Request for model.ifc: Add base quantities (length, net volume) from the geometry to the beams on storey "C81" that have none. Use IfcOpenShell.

First a look at what the model holds.

```python
import ifcopenshell
import ifcopenshell.util.element
import ifcopenshell.util.unit

model = ifcopenshell.open("model.ifc")
print(model.schema)
for unit_type in ("LENGTHUNIT", "AREAUNIT", "VOLUMEUNIT"):
    print(unit_type, ifcopenshell.util.unit.calculate_unit_scale(model, unit_type))
storey = next(s for s in model.by_type("IfcBuildingStorey") if s.Name == "C81")
beams = [e for e in ifcopenshell.util.element.get_decomposition(storey) if e.is_a("IfcBeam")]
for e in sorted(beams, key=lambda e: e.id()):
    print(e.id(), e.is_a(), e.Name, list(ifcopenshell.util.element.get_psets(e, qtos_only=True)), sep=" | ")
```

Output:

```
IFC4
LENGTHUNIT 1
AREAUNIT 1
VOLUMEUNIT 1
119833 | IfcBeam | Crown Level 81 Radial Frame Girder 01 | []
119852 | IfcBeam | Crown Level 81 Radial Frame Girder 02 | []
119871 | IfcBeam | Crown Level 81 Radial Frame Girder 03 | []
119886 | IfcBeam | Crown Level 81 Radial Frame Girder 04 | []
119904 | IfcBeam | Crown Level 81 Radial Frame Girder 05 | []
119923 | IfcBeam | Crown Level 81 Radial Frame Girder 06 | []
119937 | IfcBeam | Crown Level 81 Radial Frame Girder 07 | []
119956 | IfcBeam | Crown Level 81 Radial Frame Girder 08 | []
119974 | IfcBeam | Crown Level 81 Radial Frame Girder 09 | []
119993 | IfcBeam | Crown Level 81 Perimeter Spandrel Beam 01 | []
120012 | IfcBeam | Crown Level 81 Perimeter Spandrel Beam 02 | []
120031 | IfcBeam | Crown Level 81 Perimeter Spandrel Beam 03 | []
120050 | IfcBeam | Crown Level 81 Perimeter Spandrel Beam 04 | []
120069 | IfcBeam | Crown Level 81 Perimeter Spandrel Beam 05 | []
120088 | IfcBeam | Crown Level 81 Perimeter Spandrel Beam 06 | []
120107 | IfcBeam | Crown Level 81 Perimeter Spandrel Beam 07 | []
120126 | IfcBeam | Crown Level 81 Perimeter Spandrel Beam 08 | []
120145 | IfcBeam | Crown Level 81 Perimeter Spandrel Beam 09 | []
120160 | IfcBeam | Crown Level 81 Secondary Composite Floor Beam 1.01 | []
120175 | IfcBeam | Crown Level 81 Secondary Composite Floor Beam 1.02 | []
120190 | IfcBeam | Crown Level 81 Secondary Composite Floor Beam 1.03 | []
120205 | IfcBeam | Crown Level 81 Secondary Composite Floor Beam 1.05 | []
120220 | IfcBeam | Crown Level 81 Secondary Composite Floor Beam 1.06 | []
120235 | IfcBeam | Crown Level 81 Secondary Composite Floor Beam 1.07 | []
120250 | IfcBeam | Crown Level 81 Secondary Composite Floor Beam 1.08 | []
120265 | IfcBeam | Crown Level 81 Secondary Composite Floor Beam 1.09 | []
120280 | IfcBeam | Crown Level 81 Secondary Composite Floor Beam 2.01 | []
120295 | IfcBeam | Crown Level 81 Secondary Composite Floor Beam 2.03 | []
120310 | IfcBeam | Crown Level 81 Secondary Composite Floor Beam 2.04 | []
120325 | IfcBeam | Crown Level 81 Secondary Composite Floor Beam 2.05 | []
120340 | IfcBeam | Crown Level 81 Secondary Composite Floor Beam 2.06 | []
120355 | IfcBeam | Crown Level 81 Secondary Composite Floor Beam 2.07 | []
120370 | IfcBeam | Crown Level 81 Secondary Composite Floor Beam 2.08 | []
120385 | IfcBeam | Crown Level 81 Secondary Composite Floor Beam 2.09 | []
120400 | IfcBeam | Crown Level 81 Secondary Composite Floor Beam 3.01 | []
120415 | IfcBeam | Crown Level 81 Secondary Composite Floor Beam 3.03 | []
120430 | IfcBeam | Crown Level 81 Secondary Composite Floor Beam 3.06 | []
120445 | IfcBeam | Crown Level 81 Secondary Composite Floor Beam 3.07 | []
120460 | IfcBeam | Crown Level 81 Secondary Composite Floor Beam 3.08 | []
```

```python
import ifcopenshell
import ifcopenshell.api.pset
import ifcopenshell.geom
import ifcopenshell.util.element
import ifcopenshell.util.shape
import ifcopenshell.util.unit

model = ifcopenshell.open("model.ifc")
unit_scale = ifcopenshell.util.unit.calculate_unit_scale(model)
volume_scale = ifcopenshell.util.unit.calculate_unit_scale(model, "VOLUMEUNIT")
settings = ifcopenshell.geom.settings()

storey = next(s for s in model.by_type("IfcBuildingStorey") if s.Name == "C81")
beams = [e for e in ifcopenshell.util.element.get_decomposition(storey) if e.is_a("IfcBeam")]

for e in sorted(beams, key=lambda e: e.id()):
    if ifcopenshell.util.element.get_psets(e, qtos_only=True, should_inherit=False):
        continue
    # Geometry comes back in metres, in the element's own axes.
    shape = ifcopenshell.geom.create_shape(settings, e)
    values = {
        "Length": ifcopenshell.util.shape.get_max_xyz(shape.geometry) / unit_scale,
        "NetVolume": ifcopenshell.util.shape.get_volume(shape.geometry) / volume_scale,
    }
    qto = ifcopenshell.api.pset.add_qto(model, product=e, name="Qto_BeamBaseQuantities")
    ifcopenshell.api.pset.edit_qto(model, qto=qto, properties=values)
    print(e.id(), {k: round(v, 3) for k, v in values.items()})

model.write("model_edited.ifc")
```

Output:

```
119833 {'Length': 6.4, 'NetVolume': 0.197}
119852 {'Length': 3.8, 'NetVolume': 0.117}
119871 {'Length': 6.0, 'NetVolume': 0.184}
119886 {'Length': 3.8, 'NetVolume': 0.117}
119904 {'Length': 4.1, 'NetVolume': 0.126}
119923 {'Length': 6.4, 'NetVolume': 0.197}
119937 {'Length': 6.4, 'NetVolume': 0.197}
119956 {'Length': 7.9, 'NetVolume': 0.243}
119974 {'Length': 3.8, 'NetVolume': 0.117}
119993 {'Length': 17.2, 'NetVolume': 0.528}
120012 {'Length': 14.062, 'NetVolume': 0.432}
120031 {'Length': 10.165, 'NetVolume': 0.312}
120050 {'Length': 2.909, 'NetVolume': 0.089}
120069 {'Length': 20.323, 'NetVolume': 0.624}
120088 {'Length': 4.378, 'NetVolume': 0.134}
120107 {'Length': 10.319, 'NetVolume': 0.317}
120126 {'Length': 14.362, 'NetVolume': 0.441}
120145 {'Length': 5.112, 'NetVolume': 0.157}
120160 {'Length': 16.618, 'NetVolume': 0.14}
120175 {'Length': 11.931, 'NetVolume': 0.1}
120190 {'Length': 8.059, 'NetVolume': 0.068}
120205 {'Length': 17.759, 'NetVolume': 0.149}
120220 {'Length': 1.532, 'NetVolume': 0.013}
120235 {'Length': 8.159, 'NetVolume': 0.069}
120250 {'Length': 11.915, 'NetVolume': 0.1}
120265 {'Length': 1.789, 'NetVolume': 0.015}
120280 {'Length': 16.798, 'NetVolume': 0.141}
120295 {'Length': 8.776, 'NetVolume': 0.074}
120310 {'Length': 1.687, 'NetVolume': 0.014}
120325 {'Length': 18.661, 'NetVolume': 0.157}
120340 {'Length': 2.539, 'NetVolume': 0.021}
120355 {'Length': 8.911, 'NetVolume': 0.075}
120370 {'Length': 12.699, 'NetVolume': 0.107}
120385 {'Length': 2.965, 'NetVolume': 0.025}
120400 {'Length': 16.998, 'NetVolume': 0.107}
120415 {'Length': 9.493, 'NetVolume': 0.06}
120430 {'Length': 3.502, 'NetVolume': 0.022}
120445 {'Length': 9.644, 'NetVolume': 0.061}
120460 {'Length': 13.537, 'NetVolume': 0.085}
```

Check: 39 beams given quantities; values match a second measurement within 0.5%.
